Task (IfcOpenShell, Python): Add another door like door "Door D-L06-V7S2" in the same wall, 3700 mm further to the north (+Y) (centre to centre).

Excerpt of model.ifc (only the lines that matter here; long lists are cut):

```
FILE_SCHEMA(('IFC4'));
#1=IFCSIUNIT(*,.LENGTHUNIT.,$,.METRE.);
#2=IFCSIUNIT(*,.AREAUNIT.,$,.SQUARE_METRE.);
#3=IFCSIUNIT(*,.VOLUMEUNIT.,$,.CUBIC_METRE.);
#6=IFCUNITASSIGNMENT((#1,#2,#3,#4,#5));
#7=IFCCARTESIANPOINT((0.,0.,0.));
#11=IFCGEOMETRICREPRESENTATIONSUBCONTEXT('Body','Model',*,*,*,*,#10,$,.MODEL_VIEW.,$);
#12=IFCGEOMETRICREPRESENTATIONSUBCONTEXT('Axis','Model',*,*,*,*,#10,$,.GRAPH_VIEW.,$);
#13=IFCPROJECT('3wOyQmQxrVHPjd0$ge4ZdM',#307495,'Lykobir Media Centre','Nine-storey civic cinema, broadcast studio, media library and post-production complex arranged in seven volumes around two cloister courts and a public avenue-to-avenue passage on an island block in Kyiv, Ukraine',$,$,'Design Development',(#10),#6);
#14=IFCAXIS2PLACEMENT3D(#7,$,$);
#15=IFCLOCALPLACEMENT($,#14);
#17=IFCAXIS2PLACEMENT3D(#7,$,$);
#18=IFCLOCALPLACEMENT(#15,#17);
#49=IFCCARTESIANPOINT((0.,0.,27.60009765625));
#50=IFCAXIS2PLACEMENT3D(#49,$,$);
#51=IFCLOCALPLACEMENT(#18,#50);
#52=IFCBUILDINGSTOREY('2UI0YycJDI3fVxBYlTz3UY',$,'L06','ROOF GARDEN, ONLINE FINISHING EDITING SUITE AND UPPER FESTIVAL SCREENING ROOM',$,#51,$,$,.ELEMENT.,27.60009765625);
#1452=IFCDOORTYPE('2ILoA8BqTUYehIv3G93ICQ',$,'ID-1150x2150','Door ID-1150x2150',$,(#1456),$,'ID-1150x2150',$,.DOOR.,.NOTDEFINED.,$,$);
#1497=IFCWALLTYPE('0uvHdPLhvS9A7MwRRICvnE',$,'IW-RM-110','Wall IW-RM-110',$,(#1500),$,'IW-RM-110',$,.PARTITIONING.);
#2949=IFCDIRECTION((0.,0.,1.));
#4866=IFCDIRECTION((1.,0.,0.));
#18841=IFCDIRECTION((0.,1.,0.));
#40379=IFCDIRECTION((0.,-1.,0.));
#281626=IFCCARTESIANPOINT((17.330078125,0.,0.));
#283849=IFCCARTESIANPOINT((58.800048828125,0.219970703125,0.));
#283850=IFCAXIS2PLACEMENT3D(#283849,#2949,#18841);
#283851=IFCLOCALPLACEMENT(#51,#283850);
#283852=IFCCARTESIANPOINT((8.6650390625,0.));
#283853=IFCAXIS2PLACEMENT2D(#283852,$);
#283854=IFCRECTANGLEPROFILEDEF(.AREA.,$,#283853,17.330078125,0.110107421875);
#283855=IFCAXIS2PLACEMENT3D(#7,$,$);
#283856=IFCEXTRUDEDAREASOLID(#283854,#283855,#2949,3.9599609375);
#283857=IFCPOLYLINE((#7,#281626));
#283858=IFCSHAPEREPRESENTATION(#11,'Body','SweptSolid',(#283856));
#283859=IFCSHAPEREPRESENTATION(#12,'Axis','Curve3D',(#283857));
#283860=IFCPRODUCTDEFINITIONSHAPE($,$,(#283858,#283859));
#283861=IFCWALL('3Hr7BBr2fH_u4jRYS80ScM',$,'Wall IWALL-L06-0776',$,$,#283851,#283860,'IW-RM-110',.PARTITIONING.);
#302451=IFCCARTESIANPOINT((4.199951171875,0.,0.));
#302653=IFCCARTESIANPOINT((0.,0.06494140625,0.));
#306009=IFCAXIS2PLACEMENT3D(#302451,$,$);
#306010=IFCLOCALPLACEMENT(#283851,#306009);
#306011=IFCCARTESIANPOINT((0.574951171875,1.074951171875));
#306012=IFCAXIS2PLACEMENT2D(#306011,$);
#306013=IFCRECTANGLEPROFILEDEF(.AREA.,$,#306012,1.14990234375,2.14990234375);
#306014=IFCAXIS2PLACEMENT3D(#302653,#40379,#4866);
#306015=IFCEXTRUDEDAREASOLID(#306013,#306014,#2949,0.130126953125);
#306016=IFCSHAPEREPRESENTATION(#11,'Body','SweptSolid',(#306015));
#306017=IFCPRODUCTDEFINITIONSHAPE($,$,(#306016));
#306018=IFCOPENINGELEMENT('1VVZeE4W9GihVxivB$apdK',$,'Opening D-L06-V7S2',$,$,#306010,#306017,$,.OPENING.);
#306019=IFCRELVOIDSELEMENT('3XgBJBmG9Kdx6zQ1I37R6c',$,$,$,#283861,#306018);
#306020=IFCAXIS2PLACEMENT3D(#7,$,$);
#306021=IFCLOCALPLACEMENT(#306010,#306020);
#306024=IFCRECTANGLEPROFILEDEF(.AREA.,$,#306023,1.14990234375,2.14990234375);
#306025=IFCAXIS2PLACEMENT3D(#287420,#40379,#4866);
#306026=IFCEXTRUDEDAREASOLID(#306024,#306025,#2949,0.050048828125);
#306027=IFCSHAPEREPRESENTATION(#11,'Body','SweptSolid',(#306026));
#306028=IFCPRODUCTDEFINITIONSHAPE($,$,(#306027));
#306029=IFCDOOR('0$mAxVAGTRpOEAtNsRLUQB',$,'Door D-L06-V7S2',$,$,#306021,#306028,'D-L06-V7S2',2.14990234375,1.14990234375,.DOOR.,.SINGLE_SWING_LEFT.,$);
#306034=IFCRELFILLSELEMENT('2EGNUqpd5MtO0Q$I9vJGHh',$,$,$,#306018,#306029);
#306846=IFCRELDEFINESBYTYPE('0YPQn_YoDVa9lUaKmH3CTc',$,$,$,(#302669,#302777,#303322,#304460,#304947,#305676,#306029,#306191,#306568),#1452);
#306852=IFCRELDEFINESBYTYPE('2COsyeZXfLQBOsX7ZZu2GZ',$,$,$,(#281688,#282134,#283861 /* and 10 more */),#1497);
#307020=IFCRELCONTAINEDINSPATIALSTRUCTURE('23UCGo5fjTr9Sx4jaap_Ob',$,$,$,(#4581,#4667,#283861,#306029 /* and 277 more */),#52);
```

```python
import ifcopenshell
import ifcopenshell.api.feature
import ifcopenshell.api.geometry
import ifcopenshell.api.root
import ifcopenshell.geom
import ifcopenshell.util.element
import ifcopenshell.util.placement
import ifcopenshell.util.shape
import ifcopenshell.util.unit

model = ifcopenshell.open("model.ifc")
unit_scale = ifcopenshell.util.unit.calculate_unit_scale(model)
settings = ifcopenshell.geom.settings()


def volume(element):
    """Net volume in cubic metres, openings subtracted."""
    shape = ifcopenshell.geom.create_shape(settings, element)
    return ifcopenshell.util.shape.get_volume(shape.geometry)


door = model.by_guid("0$mAxVAGTRpOEAtNsRLUQB")
opening = door.FillsVoids[0].RelatingOpeningElement
wall = opening.VoidsElements[0].RelatingBuildingElement
before = volume(wall)
shift = ifcopenshell.util.placement.get_local_placement(wall.ObjectPlacement)[:3, 0] * 3.7 / unit_scale

# copy_class copies the void relationship, type, container and properties, but no geometry.
new_opening = ifcopenshell.api.root.copy_class(model, product=opening)
new_opening.Representation = ifcopenshell.util.element.copy_deep(
    model, opening.Representation, exclude=["IfcGeometricRepresentationContext", "IfcRepresentationMap"]
)
new_door = ifcopenshell.api.root.copy_class(model, product=door)
new_door.Representation = ifcopenshell.util.element.copy_deep(
    model, door.Representation, exclude=["IfcGeometricRepresentationContext", "IfcRepresentationMap"]
)
new_door.Tag = None
ifcopenshell.api.feature.add_filling(model, opening=new_opening, element=new_door)

for old, new in ((opening, new_opening), (door, new_door)):
    matrix = ifcopenshell.util.placement.get_local_placement(old.ObjectPlacement)
    matrix[:3, 3] += shift
    ifcopenshell.api.geometry.edit_object_placement(model, product=new, matrix=matrix, is_si=False)

after = volume(wall)

print(f"wall volume {before:.3f} -> {after:.3f} m3")

model.write("model_edited.ifc")
```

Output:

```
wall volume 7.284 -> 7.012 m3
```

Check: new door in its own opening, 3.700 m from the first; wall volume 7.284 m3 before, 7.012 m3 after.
